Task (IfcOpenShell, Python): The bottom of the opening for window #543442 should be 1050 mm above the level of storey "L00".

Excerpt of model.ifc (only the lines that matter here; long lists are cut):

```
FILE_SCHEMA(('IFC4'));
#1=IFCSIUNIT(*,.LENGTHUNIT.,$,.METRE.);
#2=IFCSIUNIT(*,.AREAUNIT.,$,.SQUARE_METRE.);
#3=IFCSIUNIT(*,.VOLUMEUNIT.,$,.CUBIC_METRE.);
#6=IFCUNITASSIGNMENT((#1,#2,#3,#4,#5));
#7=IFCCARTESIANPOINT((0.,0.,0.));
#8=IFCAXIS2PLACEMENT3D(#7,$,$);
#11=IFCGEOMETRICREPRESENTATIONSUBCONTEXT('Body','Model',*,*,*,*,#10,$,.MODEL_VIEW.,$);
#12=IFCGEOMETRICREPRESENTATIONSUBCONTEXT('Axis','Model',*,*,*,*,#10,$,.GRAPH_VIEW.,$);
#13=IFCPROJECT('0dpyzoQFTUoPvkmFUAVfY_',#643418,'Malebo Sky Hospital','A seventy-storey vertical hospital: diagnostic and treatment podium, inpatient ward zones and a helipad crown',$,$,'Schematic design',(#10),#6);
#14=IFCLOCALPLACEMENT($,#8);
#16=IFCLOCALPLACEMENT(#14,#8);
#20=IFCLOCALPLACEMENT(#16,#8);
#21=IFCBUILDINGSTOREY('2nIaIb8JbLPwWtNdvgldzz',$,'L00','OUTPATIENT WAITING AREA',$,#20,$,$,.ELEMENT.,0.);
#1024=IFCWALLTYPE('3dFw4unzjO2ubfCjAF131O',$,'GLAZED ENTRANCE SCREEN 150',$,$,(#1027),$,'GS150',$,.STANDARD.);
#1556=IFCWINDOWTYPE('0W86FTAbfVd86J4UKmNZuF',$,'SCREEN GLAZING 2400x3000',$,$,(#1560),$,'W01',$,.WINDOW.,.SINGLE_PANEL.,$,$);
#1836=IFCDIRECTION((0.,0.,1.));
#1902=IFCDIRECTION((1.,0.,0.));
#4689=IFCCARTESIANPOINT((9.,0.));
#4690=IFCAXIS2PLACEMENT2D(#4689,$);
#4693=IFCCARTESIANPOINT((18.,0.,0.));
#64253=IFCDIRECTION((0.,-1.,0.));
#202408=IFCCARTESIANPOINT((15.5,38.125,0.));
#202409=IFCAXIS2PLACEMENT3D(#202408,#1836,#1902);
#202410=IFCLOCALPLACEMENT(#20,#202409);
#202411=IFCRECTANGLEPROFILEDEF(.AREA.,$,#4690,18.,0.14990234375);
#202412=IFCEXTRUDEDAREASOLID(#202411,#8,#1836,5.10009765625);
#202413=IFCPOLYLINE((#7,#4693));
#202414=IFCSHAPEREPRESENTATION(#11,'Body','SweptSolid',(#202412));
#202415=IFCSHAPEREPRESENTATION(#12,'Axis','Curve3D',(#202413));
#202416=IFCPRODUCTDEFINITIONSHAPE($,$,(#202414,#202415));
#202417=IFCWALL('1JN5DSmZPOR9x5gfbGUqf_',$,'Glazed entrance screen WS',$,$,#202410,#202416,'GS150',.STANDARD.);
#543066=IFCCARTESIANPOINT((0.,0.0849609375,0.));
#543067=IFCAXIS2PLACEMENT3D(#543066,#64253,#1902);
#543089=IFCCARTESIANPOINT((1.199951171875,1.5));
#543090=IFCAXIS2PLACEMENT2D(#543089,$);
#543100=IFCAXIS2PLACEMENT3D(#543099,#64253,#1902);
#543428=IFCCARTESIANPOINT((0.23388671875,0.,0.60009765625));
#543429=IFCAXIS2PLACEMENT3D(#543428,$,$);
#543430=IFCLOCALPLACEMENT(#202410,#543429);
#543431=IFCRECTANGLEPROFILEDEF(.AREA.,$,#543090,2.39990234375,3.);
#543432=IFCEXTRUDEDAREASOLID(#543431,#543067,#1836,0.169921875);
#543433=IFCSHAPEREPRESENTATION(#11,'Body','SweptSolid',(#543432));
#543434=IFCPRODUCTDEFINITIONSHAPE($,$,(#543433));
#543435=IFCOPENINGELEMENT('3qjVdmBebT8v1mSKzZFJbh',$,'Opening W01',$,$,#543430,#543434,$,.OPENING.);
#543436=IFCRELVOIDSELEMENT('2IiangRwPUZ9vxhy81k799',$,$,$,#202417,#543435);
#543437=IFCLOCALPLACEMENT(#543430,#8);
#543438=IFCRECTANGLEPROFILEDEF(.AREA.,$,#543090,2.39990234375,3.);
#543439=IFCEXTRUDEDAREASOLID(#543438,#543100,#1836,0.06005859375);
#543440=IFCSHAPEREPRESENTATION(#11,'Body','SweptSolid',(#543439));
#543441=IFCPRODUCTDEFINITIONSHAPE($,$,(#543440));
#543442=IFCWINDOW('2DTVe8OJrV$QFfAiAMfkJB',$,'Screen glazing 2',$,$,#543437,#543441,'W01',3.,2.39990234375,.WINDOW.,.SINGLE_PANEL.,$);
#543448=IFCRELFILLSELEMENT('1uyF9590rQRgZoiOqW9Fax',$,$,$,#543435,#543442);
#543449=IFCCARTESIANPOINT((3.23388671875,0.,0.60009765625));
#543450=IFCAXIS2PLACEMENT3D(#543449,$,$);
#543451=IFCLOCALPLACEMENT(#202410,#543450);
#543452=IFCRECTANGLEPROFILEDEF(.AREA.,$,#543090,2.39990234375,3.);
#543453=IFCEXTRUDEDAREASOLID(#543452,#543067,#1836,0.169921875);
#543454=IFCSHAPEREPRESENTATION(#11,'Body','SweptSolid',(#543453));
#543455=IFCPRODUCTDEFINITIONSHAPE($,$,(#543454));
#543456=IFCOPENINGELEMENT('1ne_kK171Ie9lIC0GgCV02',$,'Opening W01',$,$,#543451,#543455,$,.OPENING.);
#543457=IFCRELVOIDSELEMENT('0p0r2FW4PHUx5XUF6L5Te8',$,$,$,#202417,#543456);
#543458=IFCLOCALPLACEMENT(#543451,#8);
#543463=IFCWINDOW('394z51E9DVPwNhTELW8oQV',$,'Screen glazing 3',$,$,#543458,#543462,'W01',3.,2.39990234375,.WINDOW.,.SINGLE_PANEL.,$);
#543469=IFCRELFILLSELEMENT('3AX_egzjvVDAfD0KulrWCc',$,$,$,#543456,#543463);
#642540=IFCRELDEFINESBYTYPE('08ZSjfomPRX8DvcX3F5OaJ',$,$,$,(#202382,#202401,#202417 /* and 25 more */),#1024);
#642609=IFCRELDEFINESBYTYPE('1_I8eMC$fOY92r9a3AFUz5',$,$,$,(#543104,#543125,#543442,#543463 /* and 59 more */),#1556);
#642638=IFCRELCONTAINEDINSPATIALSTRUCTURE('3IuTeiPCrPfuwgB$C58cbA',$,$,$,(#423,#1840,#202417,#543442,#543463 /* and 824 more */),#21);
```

```python
import numpy as np
import ifcopenshell
import ifcopenshell.api.geometry
import ifcopenshell.geom
import ifcopenshell.util.element
import ifcopenshell.util.placement
import ifcopenshell.util.shape
import ifcopenshell.util.unit

model = ifcopenshell.open("model.ifc")
unit_scale = ifcopenshell.util.unit.calculate_unit_scale(model)

window = model.by_id(543442)
opening = window.FillsVoids[0].RelatingOpeningElement
storey = ifcopenshell.util.element.get_container(window, ifc_class="IfcBuildingStorey")
level = ifcopenshell.util.placement.get_local_placement(storey.ObjectPlacement)[2, 3]

# The opening's origin need not be at the sill, so measure its lowest point.
shape = ifcopenshell.geom.create_shape(ifcopenshell.geom.settings(), opening)
bottom = ifcopenshell.util.shape.get_shape_bottom_elevation(shape, shape.geometry) / unit_scale
dz = level + 1.05 - bottom

shift = np.array([0.0, 0.0, dz])
# The window is placed relative to its opening, so it follows when the opening moves.
matrix = ifcopenshell.util.placement.get_local_placement(opening.ObjectPlacement)
matrix[:3, 3] += shift
ifcopenshell.api.geometry.edit_object_placement(
    model, product=opening, matrix=matrix, is_si=False, should_transform_children=True
)

print(f"moved by {dz * unit_scale:+.3f} m")

model.write("model_rev.ifc")
```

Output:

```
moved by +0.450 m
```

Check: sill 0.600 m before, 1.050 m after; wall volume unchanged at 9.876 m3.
